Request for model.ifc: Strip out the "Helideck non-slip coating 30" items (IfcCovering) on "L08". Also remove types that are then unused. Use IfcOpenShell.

First a look at what the model holds.

```python
import ifcopenshell
import ifcopenshell.util.element

model = ifcopenshell.open("model.ifc")
print(model.schema)
storey = next(s for s in model.by_type("IfcBuildingStorey") if s.Name == "L08")
coverings = [e for e in ifcopenshell.util.element.get_decomposition(storey) if e.is_a("IfcCovering")]
seen = {}
for e in coverings:
    element_type = ifcopenshell.util.element.get_type(e)
    name = element_type.Name if element_type not in (None, e) else None
    seen[name] = seen.get(name, 0) + 1
for name, count in sorted(seen.items(), key=str):
    print(count, "x", name)
```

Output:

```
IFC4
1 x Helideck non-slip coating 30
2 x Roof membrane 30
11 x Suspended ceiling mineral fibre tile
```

```python
import ifcopenshell
import ifcopenshell.api.root
import ifcopenshell.util.element

model = ifcopenshell.open("model.ifc")

storey = next(s for s in model.by_type("IfcBuildingStorey") if s.Name == "L08")
coverings = [e for e in ifcopenshell.util.element.get_decomposition(storey) if e.is_a("IfcCovering")]
targets = [e for e in coverings if (t := ifcopenshell.util.element.get_type(e)) not in (None, e) and t.Name == "Helideck non-slip coating 30"]
types = {ifcopenshell.util.element.get_type(e) for e in targets} - {None, *targets}

for e in targets:
    ifcopenshell.api.root.remove_product(model, product=e)
print(len(targets), "removed")

unused = [t for t in types if not ifcopenshell.util.element.get_types(t)]
for t in unused:
    ifcopenshell.api.root.remove_product(model, product=t)
print(len(unused), "unused types removed")

model.write("model_rev.ifc")
```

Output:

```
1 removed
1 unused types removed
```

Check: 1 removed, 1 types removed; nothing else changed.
